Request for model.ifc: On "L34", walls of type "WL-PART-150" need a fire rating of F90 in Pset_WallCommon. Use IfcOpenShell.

First a look at what the model holds.

```python
import ifcopenshell
import ifcopenshell.util.element

model = ifcopenshell.open("model.ifc")
print(model.schema)
storey = next(s for s in model.by_type("IfcBuildingStorey") if s.Name == "L34")
walls = [e for e in ifcopenshell.util.element.get_decomposition(storey) if e.is_a("IfcWall")]
seen = {}
for e in walls:
    element_type = ifcopenshell.util.element.get_type(e)
    key = (element_type.Name if element_type != e and element_type else None, ifcopenshell.util.element.get_pset(e, "Pset_WallCommon", "FireRating"))
    seen[key] = seen.get(key, 0) + 1
for (name, value), count in sorted(seen.items(), key=str):
    print(count, "x", name, "|", value)
```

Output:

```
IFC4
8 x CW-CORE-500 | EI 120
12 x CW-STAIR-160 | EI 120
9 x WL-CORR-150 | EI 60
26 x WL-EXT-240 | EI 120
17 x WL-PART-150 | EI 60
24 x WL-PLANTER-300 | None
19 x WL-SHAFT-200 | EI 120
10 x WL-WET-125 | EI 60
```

```python
import ifcopenshell
import ifcopenshell.api.pset
import ifcopenshell.util.element

model = ifcopenshell.open("model.ifc")

storey = next(s for s in model.by_type("IfcBuildingStorey") if s.Name == "L34")
walls = [e for e in ifcopenshell.util.element.get_decomposition(storey) if e.is_a("IfcWall")]

count = 0
for e in walls:
    element_type = ifcopenshell.util.element.get_type(e)
    if element_type in (None, e) or element_type.Name != "WL-PART-150":
        continue
    found = ifcopenshell.util.element.get_pset(e, "Pset_WallCommon", should_inherit=False)
    if found:
        pset = model.by_id(found["id"])
        if len(ifcopenshell.util.element.get_elements_by_pset(pset)) > 1:
            pset = ifcopenshell.api.pset.unshare_pset(model, products=[e], pset=pset)[0]
    else:
        pset = ifcopenshell.api.pset.add_pset(model, product=e, name="Pset_WallCommon")
    ifcopenshell.api.pset.edit_pset(model, pset=pset, properties={"FireRating": "F90"})
    count += 1

print(count, "walls updated")

model.write("model_v2.ifc")
```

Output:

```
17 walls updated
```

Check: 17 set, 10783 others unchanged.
